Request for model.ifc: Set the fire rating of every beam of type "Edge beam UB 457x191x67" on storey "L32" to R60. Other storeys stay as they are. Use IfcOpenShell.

First a look at what the model holds.

```python
import ifcopenshell
import ifcopenshell.util.element

model = ifcopenshell.open("model.ifc")
print(model.schema)
storey = next(s for s in model.by_type("IfcBuildingStorey") if s.Name == "L32")
beams = [e for e in ifcopenshell.util.element.get_decomposition(storey) if e.is_a("IfcBeam")]
seen = {}
for e in beams:
    element_type = ifcopenshell.util.element.get_type(e)
    key = (element_type.Name if element_type != e and element_type else None, ifcopenshell.util.element.get_pset(e, "Pset_BeamCommon", "FireRating"))
    seen[key] = seen.get(key, 0) + 1
for (name, value), count in sorted(seen.items(), key=str):
    print(count, "x", name, "|", value)
```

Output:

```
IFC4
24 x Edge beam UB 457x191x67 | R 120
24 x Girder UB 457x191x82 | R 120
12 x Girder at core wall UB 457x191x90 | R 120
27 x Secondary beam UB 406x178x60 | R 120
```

```python
import ifcopenshell
import ifcopenshell.api.pset
import ifcopenshell.util.element

model = ifcopenshell.open("model.ifc")

storey = next(s for s in model.by_type("IfcBuildingStorey") if s.Name == "L32")
beams = [e for e in ifcopenshell.util.element.get_decomposition(storey) if e.is_a("IfcBeam")]

count = 0
for e in beams:
    element_type = ifcopenshell.util.element.get_type(e)
    if element_type in (None, e) or element_type.Name != "Edge beam UB 457x191x67":
        continue
    # add_pset returns the element's existing set when there is one.
    pset = ifcopenshell.api.pset.add_pset(model, product=e, name="Pset_BeamCommon")
    ifcopenshell.api.pset.edit_pset(model, pset=pset, properties={"FireRating": "R60"})
    count += 1

print(count, "beams updated")

model.write("model_rev.ifc")
```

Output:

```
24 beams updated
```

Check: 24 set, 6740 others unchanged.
